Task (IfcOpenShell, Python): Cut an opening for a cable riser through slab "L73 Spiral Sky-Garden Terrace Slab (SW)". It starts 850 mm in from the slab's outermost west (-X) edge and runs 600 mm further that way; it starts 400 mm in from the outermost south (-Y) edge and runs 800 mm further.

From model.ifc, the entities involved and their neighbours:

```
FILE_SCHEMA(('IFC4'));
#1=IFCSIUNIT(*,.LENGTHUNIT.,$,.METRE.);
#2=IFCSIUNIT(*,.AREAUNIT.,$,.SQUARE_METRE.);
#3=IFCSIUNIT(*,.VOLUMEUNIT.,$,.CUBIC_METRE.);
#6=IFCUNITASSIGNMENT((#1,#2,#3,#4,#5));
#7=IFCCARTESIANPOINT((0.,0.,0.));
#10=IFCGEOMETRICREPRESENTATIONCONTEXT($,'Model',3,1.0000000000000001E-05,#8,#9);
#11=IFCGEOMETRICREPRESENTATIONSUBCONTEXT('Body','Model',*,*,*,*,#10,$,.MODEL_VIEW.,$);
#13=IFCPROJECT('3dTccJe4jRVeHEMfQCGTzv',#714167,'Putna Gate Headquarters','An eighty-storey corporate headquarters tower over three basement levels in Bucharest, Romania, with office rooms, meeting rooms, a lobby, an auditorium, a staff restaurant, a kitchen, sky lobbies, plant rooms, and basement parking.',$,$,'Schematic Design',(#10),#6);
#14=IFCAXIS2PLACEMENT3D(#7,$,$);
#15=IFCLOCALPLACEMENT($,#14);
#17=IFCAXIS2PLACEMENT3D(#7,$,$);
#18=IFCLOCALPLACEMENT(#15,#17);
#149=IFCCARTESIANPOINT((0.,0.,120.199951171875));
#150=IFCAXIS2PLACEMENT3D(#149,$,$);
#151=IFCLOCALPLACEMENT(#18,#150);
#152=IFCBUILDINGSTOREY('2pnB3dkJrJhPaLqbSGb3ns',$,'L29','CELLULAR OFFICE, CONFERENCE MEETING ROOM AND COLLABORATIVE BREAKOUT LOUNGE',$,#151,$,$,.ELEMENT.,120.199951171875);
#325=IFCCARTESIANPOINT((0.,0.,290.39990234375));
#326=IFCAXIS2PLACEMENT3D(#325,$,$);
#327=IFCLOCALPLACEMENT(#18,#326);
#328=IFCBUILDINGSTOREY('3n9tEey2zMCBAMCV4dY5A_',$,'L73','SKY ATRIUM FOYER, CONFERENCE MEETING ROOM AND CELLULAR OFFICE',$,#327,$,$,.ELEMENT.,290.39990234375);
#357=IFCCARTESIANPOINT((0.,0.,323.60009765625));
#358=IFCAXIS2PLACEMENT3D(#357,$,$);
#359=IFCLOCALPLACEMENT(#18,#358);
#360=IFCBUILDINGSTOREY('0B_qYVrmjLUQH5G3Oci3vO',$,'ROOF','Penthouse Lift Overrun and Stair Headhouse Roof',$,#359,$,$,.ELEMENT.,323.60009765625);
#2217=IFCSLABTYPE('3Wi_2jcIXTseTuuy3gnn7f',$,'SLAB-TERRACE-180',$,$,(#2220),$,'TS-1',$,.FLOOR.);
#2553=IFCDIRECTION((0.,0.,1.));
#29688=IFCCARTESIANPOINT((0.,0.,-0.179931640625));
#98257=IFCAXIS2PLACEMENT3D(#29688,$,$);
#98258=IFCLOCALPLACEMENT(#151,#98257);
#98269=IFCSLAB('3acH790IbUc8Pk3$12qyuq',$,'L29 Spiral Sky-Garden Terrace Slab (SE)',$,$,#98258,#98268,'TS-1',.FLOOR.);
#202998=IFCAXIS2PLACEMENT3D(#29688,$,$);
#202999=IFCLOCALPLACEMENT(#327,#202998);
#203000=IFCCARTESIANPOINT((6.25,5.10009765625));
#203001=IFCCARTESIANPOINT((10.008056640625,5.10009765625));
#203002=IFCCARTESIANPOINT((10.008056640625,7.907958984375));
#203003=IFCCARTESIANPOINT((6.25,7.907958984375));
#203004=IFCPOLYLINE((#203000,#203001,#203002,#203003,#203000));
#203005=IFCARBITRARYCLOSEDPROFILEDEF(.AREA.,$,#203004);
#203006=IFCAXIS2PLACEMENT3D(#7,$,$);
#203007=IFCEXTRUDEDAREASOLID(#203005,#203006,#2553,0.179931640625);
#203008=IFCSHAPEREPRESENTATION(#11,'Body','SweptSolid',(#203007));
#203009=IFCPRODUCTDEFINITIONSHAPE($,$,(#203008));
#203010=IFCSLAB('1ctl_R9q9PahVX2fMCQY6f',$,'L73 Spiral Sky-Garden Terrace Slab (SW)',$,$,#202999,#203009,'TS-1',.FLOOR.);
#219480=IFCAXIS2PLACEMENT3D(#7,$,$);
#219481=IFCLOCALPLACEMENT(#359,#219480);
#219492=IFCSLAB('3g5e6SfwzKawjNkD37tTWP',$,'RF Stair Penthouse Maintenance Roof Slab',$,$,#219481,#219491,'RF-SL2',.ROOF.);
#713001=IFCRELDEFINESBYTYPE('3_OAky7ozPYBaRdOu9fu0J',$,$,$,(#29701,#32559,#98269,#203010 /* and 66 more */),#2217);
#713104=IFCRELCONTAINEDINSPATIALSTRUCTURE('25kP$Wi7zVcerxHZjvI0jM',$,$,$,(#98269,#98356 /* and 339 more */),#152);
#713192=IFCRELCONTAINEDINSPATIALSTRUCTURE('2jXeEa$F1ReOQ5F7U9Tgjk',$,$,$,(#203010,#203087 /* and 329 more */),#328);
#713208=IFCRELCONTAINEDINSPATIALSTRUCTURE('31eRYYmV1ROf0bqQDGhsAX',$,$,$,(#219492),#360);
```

```python
import numpy as np
import ifcopenshell
import ifcopenshell.api.feature
import ifcopenshell.api.geometry
import ifcopenshell.api.root
import ifcopenshell.geom
import ifcopenshell.util.placement
import ifcopenshell.util.representation
import ifcopenshell.util.shape
import ifcopenshell.util.unit

model = ifcopenshell.open("model.ifc")
unit_scale = ifcopenshell.util.unit.calculate_unit_scale(model)
settings = ifcopenshell.geom.settings()


def volume(element):
    """Net volume in cubic metres, openings subtracted."""
    shape = ifcopenshell.geom.create_shape(settings, element)
    return ifcopenshell.util.shape.get_volume(shape.geometry)


slab = model.by_id(203010)
before = volume(slab)

# Extent in the slab's own axes, in metres. The edges named are its -X and -Y sides.
slab_shape = ifcopenshell.geom.create_shape(settings, slab)
vertices = ifcopenshell.util.shape.get_vertices(slab_shape.geometry)
x_min, y_min, bottom = vertices.min(axis=0)
top = vertices[:, 2].max()

opening = ifcopenshell.api.root.create_entity(model, ifc_class="IfcOpeningElement", name="Cable riser opening", predefined_type="OPENING")
context = ifcopenshell.util.representation.get_context(model, "Model", "Body", "MODEL_VIEW")
width, depth = 0.6, 0.8
outline = [(0.0, 0.0), (width, 0.0), (width, depth), (0.0, depth), (0.0, 0.0)]
# Overshoot both faces by 50 mm so the cut is clean.
shape = ifcopenshell.api.geometry.add_slab_representation(
    model, context=context, depth=top - bottom + 0.1, polyline=outline
)
ifcopenshell.api.geometry.assign_representation(model, product=opening, representation=shape)

matrix = ifcopenshell.util.placement.get_local_placement(slab.ObjectPlacement)
matrix[:, 3] = matrix @ np.append(np.array([x_min + 0.85, y_min + 0.4, bottom - 0.05]) / unit_scale, 1.0)
ifcopenshell.api.geometry.edit_object_placement(model, product=opening, matrix=matrix, is_si=False)
ifcopenshell.api.feature.add_feature(model, feature=opening, element=slab)

after = volume(slab)

print(f"slab volume {before:.3f} -> {after:.3f} m3")

model.write("model_rev.ifc")
```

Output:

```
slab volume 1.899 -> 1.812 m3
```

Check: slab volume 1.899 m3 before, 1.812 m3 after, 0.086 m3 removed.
